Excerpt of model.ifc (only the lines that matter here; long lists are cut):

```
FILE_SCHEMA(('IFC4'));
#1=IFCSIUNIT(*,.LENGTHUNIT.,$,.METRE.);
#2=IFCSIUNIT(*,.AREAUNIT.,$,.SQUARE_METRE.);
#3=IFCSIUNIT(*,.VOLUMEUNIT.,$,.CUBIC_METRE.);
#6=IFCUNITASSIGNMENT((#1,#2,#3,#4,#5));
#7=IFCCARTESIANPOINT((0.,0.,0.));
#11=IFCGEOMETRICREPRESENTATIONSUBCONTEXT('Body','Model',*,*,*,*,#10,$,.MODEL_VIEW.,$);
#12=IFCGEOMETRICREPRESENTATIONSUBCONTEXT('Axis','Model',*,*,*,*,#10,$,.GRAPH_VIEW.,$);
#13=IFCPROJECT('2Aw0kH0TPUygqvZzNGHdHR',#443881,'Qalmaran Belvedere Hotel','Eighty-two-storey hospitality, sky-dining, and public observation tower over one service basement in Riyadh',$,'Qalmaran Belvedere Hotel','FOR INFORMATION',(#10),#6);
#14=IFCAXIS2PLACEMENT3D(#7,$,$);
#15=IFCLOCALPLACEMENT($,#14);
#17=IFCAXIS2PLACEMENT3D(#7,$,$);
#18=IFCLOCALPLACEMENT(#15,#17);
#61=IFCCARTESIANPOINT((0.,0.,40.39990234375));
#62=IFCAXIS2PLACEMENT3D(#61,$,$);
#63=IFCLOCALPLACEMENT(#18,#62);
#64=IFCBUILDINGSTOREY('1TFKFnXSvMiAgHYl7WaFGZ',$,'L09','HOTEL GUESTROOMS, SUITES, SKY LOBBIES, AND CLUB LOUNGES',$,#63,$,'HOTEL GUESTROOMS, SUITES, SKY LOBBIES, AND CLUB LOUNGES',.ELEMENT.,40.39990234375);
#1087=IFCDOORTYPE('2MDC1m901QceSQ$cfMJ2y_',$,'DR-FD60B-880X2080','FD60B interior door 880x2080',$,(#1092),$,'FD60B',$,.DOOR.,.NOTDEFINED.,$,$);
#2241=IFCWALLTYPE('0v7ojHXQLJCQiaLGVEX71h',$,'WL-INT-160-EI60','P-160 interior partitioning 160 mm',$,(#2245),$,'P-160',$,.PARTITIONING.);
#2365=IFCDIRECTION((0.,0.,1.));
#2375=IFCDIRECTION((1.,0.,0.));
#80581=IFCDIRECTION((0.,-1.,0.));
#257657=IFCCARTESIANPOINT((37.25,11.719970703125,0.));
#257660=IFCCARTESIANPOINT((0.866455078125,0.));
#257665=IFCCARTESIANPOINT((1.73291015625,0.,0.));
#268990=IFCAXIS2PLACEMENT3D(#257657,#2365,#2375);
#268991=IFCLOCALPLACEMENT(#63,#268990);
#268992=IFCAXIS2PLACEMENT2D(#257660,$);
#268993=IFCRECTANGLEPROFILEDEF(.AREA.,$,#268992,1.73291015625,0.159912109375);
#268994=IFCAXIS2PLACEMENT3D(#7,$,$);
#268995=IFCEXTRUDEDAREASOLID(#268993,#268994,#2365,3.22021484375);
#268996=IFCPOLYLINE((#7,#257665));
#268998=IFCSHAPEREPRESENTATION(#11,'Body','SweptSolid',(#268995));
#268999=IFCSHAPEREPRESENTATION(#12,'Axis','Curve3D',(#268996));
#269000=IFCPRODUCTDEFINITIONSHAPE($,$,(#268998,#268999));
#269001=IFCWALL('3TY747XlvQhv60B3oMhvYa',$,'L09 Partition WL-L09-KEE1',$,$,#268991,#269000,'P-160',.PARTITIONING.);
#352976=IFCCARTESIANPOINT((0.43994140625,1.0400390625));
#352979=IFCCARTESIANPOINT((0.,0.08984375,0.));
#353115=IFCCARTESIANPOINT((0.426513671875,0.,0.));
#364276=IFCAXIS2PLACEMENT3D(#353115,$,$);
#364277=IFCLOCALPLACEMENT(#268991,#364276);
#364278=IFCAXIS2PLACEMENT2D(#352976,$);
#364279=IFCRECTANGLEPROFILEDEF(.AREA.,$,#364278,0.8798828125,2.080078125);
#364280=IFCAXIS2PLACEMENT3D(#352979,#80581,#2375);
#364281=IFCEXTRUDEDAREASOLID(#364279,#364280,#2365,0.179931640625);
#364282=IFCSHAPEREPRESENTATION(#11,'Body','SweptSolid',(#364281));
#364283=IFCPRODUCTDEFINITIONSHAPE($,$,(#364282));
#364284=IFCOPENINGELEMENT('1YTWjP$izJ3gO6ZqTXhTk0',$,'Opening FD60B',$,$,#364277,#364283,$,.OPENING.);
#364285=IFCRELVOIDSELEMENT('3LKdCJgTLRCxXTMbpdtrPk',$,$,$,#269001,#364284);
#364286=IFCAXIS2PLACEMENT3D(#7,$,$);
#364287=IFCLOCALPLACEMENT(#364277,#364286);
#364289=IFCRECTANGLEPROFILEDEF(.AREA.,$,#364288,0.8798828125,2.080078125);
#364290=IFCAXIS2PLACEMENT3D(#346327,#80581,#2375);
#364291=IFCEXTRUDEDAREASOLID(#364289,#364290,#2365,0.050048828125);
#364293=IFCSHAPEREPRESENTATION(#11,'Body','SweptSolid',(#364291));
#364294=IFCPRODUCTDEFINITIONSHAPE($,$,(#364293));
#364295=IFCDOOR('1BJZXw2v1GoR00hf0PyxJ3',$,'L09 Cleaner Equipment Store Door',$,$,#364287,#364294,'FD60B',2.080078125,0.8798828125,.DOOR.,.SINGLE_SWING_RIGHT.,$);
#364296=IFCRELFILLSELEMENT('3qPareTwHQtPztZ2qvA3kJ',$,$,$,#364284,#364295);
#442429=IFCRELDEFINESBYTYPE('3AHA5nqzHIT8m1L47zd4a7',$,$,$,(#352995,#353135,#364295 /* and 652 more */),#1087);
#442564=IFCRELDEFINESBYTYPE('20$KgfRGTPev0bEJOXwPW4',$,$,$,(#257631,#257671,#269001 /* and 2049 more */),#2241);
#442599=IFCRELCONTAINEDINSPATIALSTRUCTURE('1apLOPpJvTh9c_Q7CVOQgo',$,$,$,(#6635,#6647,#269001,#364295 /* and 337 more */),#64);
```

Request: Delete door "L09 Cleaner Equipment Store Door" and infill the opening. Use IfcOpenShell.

```python
import ifcopenshell
import ifcopenshell.api.feature
import ifcopenshell.api.root
import ifcopenshell.geom
import ifcopenshell.util.shape

model = ifcopenshell.open("model.ifc")
settings = ifcopenshell.geom.settings()


def volume(element):
    """Net volume in cubic metres, openings subtracted."""
    shape = ifcopenshell.geom.create_shape(settings, element)
    return ifcopenshell.util.shape.get_volume(shape.geometry)


door = model.by_guid("1BJZXw2v1GoR00hf0PyxJ3")
opening = door.FillsVoids[0].RelatingOpeningElement
wall = opening.VoidsElements[0].RelatingBuildingElement
before = volume(wall)

ifcopenshell.api.root.remove_product(model, product=door)
ifcopenshell.api.feature.remove_feature(model, feature=opening)

after = volume(wall)

print(f"wall volume {before:.3f} -> {after:.3f} m3")

model.write("model-out.ifc")
```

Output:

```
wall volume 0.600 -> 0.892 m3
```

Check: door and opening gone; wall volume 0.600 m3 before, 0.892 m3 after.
